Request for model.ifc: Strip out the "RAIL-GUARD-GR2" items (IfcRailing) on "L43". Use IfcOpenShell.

First a look at what the model holds.

```python
import ifcopenshell
import ifcopenshell.util.element

model = ifcopenshell.open("model.ifc")
print(model.schema)
storey = next(s for s in model.by_type("IfcBuildingStorey") if s.Name == "L43")
railings = [e for e in ifcopenshell.util.element.get_decomposition(storey) if e.is_a("IfcRailing")]
seen = {}
for e in railings:
    element_type = ifcopenshell.util.element.get_type(e)
    name = element_type.Name if element_type not in (None, e) else None
    seen[name] = seen.get(name, 0) + 1
for name, count in sorted(seen.items(), key=str):
    print(count, "x", name)
```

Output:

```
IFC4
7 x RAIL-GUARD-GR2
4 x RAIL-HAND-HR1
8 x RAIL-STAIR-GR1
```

```python
import ifcopenshell
import ifcopenshell.api.root
import ifcopenshell.util.element

model = ifcopenshell.open("model.ifc")

storey = next(s for s in model.by_type("IfcBuildingStorey") if s.Name == "L43")
railings = [e for e in ifcopenshell.util.element.get_decomposition(storey) if e.is_a("IfcRailing")]
targets = [e for e in railings if (t := ifcopenshell.util.element.get_type(e)) not in (None, e) and t.Name == "RAIL-GUARD-GR2"]

for e in targets:
    ifcopenshell.api.root.remove_product(model, product=e)
print(len(targets), "removed")

model.write("model_v2.ifc")
```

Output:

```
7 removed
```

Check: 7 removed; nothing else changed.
